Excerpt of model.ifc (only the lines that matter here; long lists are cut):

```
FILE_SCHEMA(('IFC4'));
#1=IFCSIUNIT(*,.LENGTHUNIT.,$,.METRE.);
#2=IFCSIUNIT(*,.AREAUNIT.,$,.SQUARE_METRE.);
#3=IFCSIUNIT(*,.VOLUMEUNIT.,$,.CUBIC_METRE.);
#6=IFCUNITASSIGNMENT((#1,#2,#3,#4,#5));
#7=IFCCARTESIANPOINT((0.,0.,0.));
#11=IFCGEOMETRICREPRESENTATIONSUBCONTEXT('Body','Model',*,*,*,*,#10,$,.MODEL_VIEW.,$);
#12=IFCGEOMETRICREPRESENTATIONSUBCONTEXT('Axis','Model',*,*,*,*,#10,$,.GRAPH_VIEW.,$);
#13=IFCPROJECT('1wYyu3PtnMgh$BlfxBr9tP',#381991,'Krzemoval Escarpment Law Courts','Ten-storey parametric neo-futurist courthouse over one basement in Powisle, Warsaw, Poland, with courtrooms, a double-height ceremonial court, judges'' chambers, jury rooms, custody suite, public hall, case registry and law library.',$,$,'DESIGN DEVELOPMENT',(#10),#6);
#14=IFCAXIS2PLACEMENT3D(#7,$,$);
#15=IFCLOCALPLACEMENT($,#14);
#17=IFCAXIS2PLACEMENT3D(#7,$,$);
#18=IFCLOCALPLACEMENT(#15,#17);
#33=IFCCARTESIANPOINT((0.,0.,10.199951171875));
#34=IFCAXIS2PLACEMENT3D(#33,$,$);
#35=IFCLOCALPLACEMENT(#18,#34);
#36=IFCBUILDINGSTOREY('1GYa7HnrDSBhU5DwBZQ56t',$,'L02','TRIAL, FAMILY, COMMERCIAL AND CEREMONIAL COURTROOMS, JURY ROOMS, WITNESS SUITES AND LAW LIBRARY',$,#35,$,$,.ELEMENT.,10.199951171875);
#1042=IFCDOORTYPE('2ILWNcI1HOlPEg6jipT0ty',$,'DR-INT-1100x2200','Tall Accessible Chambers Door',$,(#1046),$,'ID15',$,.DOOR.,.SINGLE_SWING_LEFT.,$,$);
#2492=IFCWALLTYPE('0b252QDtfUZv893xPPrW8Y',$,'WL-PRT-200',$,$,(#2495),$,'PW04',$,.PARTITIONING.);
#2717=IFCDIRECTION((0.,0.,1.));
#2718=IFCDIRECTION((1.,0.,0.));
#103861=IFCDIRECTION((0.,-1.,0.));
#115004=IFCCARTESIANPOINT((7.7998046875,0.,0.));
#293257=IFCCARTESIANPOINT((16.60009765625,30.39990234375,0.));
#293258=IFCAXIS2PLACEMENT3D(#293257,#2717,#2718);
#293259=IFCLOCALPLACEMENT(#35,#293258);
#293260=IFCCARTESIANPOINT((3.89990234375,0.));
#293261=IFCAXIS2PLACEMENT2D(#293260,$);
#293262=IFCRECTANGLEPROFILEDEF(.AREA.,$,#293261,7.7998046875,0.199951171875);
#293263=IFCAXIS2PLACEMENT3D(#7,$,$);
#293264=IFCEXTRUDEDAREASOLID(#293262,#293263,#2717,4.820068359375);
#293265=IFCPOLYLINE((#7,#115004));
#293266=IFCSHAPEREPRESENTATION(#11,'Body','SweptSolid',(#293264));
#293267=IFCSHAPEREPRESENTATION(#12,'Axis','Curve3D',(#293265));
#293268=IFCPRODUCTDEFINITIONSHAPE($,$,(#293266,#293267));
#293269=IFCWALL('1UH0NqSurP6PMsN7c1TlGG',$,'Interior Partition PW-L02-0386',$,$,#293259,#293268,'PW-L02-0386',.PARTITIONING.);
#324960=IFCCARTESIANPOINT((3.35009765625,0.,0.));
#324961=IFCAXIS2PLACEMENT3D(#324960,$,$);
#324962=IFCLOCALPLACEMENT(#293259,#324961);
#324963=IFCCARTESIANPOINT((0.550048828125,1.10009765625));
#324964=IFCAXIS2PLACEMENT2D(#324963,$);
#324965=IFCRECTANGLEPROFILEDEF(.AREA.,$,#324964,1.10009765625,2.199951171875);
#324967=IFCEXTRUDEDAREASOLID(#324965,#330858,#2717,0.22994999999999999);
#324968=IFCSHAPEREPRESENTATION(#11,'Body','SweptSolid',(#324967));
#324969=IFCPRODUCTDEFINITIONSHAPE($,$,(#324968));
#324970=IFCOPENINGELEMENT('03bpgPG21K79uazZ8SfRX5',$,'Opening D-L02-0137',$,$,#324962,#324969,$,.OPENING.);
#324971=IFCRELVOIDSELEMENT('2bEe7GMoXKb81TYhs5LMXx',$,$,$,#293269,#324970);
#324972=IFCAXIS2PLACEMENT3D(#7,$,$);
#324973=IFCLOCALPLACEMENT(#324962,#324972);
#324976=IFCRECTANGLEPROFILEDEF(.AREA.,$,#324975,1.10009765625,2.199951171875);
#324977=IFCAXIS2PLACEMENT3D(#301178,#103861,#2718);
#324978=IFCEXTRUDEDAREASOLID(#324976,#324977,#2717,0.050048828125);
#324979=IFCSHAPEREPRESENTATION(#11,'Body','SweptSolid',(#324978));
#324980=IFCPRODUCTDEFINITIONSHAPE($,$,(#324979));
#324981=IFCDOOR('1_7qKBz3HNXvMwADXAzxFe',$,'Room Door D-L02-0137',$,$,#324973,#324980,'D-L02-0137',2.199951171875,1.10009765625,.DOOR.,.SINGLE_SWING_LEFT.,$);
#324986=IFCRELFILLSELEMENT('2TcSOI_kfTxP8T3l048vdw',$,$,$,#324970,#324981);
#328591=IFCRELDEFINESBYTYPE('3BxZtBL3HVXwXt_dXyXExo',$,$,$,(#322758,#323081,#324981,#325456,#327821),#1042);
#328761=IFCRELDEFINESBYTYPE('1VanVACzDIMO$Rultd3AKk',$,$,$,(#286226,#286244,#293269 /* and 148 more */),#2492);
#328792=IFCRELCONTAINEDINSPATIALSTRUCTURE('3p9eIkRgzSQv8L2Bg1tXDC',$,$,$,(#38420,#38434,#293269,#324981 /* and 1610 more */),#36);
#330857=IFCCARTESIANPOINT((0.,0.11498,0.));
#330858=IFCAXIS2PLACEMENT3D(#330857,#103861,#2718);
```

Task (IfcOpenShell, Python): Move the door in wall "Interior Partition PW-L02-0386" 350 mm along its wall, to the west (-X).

```python
import ifcopenshell
import ifcopenshell.api.geometry
import ifcopenshell.util.placement

model = ifcopenshell.open("model.ifc")

door = model.by_id(324981)
opening = door.FillsVoids[0].RelatingOpeningElement
wall = opening.VoidsElements[0].RelatingBuildingElement

wall_matrix = ifcopenshell.util.placement.get_local_placement(wall.ObjectPlacement)
shift = wall_matrix[:3, 0] * -0.35
before = ifcopenshell.util.placement.get_local_placement(door.ObjectPlacement)[:3, 3].copy()

# The door is placed relative to its opening, so it follows when the opening moves.
matrix = ifcopenshell.util.placement.get_local_placement(opening.ObjectPlacement)
matrix[:3, 3] += shift
ifcopenshell.api.geometry.edit_object_placement(
    model, product=opening, matrix=matrix, is_si=False, should_transform_children=True
)

after = ifcopenshell.util.placement.get_local_placement(door.ObjectPlacement)[:3, 3]
print("door moved by", (after - before).round(3) + 0.0)

model.write("model_edited.ifc")
```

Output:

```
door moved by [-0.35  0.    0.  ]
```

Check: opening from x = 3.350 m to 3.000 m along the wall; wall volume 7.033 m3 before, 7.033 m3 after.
